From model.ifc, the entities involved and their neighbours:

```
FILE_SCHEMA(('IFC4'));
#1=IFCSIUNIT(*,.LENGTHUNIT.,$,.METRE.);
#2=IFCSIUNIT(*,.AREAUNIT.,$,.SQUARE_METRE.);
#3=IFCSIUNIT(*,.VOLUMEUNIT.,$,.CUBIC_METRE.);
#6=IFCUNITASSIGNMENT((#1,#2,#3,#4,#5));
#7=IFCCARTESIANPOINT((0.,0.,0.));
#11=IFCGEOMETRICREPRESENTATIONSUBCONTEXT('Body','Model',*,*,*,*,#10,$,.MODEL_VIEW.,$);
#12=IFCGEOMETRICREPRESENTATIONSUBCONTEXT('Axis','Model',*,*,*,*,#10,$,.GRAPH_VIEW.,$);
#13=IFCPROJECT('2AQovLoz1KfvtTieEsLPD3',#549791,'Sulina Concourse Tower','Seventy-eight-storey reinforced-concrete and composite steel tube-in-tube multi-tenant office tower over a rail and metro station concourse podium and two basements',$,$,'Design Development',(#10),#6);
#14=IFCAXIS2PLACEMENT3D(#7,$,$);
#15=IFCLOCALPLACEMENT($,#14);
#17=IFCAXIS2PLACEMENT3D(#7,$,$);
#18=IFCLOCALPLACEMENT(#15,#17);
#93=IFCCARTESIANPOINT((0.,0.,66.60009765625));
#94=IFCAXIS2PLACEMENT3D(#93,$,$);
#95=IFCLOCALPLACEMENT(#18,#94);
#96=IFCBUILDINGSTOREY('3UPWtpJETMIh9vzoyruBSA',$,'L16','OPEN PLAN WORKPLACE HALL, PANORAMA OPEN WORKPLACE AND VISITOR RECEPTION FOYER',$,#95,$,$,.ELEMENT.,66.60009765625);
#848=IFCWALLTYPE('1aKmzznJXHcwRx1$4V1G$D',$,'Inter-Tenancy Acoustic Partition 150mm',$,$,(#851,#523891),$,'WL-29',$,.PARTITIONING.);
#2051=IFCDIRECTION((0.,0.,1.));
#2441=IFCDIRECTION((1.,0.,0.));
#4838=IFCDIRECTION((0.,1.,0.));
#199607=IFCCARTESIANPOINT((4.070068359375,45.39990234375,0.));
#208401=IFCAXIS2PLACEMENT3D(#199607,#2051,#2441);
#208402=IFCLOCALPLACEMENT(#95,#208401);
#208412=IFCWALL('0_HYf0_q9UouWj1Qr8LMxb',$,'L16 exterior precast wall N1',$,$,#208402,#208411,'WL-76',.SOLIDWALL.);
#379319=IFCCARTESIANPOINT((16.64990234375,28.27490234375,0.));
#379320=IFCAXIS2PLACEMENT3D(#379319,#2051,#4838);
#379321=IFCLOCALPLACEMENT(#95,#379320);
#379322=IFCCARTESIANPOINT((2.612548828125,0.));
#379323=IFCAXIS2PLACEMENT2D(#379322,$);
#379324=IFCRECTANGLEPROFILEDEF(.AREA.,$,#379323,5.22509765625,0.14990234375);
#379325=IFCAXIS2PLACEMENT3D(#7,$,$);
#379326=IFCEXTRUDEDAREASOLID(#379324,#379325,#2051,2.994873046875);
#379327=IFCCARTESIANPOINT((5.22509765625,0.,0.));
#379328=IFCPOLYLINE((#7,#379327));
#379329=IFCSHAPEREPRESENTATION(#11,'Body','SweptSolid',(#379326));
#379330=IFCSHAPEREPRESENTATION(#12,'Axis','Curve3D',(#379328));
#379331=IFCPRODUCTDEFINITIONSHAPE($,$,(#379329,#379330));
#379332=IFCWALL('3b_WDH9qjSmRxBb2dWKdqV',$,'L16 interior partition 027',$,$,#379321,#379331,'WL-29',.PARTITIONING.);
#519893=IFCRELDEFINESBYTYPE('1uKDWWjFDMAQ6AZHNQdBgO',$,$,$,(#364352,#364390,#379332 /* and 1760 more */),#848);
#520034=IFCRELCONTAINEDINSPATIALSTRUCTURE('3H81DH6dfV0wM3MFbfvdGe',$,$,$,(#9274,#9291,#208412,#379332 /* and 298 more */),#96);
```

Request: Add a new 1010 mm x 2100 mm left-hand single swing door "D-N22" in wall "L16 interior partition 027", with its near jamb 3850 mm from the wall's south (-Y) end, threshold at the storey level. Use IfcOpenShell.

```python
import numpy as np
import ifcopenshell
import ifcopenshell.api.feature
import ifcopenshell.api.geometry
import ifcopenshell.api.root
import ifcopenshell.api.spatial
import ifcopenshell.geom
import ifcopenshell.util.element
import ifcopenshell.util.placement
import ifcopenshell.util.representation
import ifcopenshell.util.shape
import ifcopenshell.util.unit

model = ifcopenshell.open("model.ifc")
unit_scale = ifcopenshell.util.unit.calculate_unit_scale(model)
settings = ifcopenshell.geom.settings()


def volume(element):
    """Net volume in cubic metres, openings subtracted."""
    shape = ifcopenshell.geom.create_shape(settings, element)
    return ifcopenshell.util.shape.get_volume(shape.geometry)


wall = model.by_guid("3b_WDH9qjSmRxBb2dWKdqV")
storey = ifcopenshell.util.element.get_container(wall, ifc_class="IfcBuildingStorey")
context = ifcopenshell.util.representation.get_context(model, "Model", "Body", "MODEL_VIEW")
before = volume(wall)

width, height, from_end, sill = 1.01, 2.1, 3.85, 0.0  # metres

# The wall runs along its own X axis, and the end named is its -X end.
wall_shape = ifcopenshell.geom.create_shape(settings, wall)
x, y, z = ifcopenshell.util.shape.get_vertices(wall_shape.geometry).T
start = x.min() + from_end
face, thickness = float(y.min()), float(y.max() - y.min())
wall_matrix = ifcopenshell.util.placement.get_local_placement(wall.ObjectPlacement)
level = ifcopenshell.util.placement.get_local_placement(storey.ObjectPlacement)[2, 3]


def in_wall(x, y):
    """Placement at x, y metres in the wall's axes, at sill height."""
    matrix = wall_matrix.copy()
    matrix[:, 3] = wall_matrix @ np.array([x / unit_scale, y / unit_scale, 0.0, 1.0])
    matrix[2, 3] = level + sill / unit_scale
    return matrix


# Opening: a box that overshoots both wall faces by 50 mm.
opening = ifcopenshell.api.root.create_entity(model, ifc_class="IfcOpeningElement", predefined_type="OPENING")
box = ifcopenshell.api.geometry.add_wall_representation(
    model, context=context, length=width, height=height, thickness=thickness + 0.1
)
ifcopenshell.api.geometry.assign_representation(model, product=opening, representation=box)
ifcopenshell.api.geometry.edit_object_placement(model, product=opening, matrix=in_wall(start, face - 0.05), is_si=False)
ifcopenshell.api.feature.add_feature(model, feature=opening, element=wall)

door = ifcopenshell.api.root.create_entity(model, ifc_class="IfcDoor", name="D-N22", predefined_type="DOOR")
door.OverallWidth, door.OverallHeight = width / unit_scale, height / unit_scale
door.OperationType = "SINGLE_SWING_LEFT"
body = ifcopenshell.api.geometry.add_door_representation(
    model,
    context=context,
    overall_width=door.OverallWidth,
    overall_height=door.OverallHeight,
    operation_type="SINGLE_SWING_LEFT",
    lining_properties={"LiningDepth": thickness / unit_scale, "ThresholdDepth": thickness / unit_scale},
)
ifcopenshell.api.geometry.assign_representation(model, product=door, representation=body)
ifcopenshell.api.spatial.assign_container(model, products=[door], relating_structure=storey)
ifcopenshell.api.feature.add_filling(model, opening=opening, element=door)

# The lining spans the wall, so the door starts at the wall face.
ifcopenshell.api.geometry.edit_object_placement(model, product=door, matrix=in_wall(start, face), is_si=False)

after = volume(wall)

print(f"wall volume {before:.3f} -> {after:.3f} m3")

model.write("model_edited.ifc")
```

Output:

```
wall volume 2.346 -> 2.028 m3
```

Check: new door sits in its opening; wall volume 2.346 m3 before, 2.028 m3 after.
